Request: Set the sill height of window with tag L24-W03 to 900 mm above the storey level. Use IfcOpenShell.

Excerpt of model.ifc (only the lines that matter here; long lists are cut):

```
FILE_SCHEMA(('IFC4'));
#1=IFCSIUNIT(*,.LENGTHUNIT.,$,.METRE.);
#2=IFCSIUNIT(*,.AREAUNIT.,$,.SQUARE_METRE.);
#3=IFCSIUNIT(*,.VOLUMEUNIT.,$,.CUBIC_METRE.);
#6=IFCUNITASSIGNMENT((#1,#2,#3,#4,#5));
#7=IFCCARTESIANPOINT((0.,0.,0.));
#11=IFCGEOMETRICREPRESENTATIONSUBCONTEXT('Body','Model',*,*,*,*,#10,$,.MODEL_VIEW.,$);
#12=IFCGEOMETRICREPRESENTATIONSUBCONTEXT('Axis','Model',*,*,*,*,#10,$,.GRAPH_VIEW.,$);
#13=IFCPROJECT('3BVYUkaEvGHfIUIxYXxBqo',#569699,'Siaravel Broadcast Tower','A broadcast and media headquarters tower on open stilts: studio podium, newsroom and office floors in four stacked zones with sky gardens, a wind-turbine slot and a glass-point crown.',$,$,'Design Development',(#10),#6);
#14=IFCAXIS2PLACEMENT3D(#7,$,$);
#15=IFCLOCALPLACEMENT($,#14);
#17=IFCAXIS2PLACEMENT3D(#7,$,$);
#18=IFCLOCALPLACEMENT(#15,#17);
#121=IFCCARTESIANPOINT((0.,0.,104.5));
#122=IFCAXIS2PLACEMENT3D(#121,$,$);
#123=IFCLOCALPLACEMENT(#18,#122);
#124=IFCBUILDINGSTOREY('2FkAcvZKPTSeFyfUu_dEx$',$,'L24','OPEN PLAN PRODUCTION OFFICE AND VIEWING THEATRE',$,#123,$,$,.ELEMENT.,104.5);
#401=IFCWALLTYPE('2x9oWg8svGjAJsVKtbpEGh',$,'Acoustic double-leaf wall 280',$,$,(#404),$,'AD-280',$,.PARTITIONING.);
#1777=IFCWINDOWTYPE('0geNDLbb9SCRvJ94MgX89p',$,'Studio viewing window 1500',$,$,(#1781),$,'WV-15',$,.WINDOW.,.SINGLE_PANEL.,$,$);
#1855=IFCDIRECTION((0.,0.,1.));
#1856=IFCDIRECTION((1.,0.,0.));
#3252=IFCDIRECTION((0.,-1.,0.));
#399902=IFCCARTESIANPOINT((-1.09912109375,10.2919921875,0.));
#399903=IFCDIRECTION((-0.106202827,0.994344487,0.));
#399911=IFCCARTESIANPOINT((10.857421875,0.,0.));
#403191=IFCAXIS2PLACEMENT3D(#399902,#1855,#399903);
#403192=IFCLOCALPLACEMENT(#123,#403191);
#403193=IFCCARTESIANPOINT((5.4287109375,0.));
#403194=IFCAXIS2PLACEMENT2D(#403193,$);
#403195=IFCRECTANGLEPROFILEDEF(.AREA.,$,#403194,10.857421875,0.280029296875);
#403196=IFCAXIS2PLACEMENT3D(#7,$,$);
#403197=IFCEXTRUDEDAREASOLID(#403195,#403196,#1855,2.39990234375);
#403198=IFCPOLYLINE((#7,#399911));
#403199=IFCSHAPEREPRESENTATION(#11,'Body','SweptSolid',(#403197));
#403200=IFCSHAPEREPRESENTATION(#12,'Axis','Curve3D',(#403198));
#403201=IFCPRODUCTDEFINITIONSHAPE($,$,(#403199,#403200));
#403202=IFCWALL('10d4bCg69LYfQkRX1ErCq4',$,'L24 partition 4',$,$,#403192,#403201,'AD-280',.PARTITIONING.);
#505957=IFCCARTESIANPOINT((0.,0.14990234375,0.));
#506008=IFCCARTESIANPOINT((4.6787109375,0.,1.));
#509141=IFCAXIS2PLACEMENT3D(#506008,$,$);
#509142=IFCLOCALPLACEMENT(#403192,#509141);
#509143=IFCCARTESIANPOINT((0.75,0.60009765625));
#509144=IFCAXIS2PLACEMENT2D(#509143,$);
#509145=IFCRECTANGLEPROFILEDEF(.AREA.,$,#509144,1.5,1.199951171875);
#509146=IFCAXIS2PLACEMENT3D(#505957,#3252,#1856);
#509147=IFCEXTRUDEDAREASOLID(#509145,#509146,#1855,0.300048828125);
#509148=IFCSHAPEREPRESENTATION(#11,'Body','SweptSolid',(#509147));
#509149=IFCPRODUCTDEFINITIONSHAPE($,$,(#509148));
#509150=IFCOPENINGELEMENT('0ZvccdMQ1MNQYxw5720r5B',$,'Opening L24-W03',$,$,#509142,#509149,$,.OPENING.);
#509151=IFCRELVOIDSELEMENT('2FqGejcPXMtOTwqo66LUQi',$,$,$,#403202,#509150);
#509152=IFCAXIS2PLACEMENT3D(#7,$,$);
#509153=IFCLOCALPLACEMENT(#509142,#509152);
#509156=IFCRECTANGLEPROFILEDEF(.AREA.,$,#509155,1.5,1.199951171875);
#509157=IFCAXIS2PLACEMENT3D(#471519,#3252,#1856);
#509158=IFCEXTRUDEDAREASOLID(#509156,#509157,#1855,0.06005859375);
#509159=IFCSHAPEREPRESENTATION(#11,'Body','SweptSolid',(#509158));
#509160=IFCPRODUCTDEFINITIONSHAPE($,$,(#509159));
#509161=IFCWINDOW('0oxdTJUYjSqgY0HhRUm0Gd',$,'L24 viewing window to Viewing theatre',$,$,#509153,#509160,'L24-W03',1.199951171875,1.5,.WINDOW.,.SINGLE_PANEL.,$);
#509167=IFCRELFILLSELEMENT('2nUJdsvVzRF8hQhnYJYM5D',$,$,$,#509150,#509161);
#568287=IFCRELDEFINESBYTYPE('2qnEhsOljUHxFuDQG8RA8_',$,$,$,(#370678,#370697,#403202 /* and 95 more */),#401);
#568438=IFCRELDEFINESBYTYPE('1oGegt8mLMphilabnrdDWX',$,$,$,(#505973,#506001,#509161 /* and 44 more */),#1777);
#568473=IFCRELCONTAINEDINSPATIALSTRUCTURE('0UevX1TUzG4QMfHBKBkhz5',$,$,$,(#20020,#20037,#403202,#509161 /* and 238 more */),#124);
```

```python
import numpy as np
import ifcopenshell
import ifcopenshell.api.geometry
import ifcopenshell.geom
import ifcopenshell.util.element
import ifcopenshell.util.placement
import ifcopenshell.util.shape
import ifcopenshell.util.unit

model = ifcopenshell.open("model.ifc")
unit_scale = ifcopenshell.util.unit.calculate_unit_scale(model)

window = model.by_id(509161)
opening = window.FillsVoids[0].RelatingOpeningElement
storey = ifcopenshell.util.element.get_container(window, ifc_class="IfcBuildingStorey")
level = ifcopenshell.util.placement.get_local_placement(storey.ObjectPlacement)[2, 3]

# The opening's origin need not be at the sill, so measure its lowest point.
shape = ifcopenshell.geom.create_shape(ifcopenshell.geom.settings(), opening)
bottom = ifcopenshell.util.shape.get_shape_bottom_elevation(shape, shape.geometry) / unit_scale
dz = level + 0.9 / unit_scale - bottom

shift = np.array([0.0, 0.0, dz])
# The window is placed relative to its opening, so it follows when the opening moves.
matrix = ifcopenshell.util.placement.get_local_placement(opening.ObjectPlacement)
matrix[:3, 3] += shift
ifcopenshell.api.geometry.edit_object_placement(
    model, product=opening, matrix=matrix, is_si=False, should_transform_children=True
)

print(f"moved by {dz * unit_scale:+.3f} m")

model.write("model_rev.ifc")
```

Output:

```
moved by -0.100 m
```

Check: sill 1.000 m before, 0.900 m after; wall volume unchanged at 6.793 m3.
